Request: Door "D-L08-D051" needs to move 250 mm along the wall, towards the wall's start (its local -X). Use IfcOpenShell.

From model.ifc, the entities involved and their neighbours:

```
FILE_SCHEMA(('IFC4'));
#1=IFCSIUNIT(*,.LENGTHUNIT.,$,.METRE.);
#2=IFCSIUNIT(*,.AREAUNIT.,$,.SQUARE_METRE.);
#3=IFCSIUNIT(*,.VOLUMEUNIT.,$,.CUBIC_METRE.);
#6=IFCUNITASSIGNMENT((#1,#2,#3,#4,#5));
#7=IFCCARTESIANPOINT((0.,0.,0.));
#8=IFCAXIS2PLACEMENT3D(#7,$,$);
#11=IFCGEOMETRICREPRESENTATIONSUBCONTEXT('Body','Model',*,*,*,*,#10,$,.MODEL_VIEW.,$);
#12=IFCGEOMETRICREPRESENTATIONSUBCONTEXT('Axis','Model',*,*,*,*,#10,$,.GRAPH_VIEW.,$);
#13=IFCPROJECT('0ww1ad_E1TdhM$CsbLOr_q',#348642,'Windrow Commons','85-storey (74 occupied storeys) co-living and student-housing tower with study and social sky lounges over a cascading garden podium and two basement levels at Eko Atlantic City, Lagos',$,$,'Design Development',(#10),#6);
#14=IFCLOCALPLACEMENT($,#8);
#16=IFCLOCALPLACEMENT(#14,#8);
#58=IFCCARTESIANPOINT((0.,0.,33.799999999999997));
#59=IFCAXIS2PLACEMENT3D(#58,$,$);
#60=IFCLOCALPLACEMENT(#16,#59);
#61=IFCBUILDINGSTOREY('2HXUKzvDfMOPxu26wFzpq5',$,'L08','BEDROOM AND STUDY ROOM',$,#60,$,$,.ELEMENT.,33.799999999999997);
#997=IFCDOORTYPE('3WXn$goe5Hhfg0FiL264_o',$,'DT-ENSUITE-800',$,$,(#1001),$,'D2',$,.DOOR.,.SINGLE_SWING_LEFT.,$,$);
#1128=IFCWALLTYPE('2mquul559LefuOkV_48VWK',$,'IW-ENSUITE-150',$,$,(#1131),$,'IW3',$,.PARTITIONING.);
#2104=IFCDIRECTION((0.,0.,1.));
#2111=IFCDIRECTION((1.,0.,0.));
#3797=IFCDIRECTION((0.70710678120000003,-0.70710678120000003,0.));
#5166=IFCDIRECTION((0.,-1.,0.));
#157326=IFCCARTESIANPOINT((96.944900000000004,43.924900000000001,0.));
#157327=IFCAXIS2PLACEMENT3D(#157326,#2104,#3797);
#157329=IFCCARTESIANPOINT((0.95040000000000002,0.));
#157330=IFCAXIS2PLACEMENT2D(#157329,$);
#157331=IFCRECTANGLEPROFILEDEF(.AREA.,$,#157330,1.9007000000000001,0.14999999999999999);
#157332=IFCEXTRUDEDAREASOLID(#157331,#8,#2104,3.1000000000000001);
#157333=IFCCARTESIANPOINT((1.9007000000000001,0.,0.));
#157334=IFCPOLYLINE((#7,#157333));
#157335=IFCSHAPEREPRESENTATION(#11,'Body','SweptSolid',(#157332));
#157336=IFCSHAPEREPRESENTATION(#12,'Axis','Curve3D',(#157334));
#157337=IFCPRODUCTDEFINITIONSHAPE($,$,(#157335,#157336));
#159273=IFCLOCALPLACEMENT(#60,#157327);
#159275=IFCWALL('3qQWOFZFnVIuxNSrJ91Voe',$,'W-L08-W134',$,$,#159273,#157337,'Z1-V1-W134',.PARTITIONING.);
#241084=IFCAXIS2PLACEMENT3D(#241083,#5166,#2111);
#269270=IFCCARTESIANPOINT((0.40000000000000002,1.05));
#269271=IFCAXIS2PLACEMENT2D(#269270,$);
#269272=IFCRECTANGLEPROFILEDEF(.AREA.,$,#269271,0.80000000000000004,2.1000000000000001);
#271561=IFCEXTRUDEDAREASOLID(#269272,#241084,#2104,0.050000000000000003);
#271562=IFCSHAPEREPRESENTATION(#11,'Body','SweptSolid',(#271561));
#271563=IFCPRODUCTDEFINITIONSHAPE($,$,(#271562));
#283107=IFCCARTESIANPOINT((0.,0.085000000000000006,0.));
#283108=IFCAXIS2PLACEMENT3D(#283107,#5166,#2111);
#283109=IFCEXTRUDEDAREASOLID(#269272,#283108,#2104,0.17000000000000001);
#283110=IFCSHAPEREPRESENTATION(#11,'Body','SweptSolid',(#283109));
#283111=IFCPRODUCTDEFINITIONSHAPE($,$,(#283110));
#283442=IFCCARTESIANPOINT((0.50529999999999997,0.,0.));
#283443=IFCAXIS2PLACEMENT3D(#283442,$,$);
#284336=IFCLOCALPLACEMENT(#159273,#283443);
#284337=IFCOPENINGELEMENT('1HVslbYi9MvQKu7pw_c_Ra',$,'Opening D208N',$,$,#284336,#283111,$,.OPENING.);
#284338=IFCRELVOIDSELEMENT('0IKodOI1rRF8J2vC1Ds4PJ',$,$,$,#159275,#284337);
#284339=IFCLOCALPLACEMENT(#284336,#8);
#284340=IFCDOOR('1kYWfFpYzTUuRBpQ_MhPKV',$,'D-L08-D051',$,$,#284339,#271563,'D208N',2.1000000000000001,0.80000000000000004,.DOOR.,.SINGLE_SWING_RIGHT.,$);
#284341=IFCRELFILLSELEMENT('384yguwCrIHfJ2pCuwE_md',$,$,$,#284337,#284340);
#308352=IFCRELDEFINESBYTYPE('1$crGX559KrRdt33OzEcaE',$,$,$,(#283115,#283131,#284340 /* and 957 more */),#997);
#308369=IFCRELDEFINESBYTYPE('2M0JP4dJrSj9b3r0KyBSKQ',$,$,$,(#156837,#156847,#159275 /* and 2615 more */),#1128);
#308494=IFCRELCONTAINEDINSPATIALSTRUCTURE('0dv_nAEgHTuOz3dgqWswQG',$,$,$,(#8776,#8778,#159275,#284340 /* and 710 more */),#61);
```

```python
import ifcopenshell
import ifcopenshell.api.geometry
import ifcopenshell.util.placement
import ifcopenshell.util.unit

model = ifcopenshell.open("model.ifc")
unit_scale = ifcopenshell.util.unit.calculate_unit_scale(model)

door = model.by_guid("1kYWfFpYzTUuRBpQ_MhPKV")
opening = door.FillsVoids[0].RelatingOpeningElement
wall = opening.VoidsElements[0].RelatingBuildingElement

wall_matrix = ifcopenshell.util.placement.get_local_placement(wall.ObjectPlacement)
shift = wall_matrix[:3, 0] * -0.25 / unit_scale
before = ifcopenshell.util.placement.get_local_placement(door.ObjectPlacement)[:3, 3].copy()

# The door is placed relative to its opening, so it follows when the opening moves.
matrix = ifcopenshell.util.placement.get_local_placement(opening.ObjectPlacement)
matrix[:3, 3] += shift
ifcopenshell.api.geometry.edit_object_placement(
    model, product=opening, matrix=matrix, is_si=False, should_transform_children=True
)

after = ifcopenshell.util.placement.get_local_placement(door.ObjectPlacement)[:3, 3]
print("door moved by", (after - before).round(3) + 0.0)

model.write("model_updated.ifc")
```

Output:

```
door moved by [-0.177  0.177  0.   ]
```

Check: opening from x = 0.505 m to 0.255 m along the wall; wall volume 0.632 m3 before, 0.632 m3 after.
